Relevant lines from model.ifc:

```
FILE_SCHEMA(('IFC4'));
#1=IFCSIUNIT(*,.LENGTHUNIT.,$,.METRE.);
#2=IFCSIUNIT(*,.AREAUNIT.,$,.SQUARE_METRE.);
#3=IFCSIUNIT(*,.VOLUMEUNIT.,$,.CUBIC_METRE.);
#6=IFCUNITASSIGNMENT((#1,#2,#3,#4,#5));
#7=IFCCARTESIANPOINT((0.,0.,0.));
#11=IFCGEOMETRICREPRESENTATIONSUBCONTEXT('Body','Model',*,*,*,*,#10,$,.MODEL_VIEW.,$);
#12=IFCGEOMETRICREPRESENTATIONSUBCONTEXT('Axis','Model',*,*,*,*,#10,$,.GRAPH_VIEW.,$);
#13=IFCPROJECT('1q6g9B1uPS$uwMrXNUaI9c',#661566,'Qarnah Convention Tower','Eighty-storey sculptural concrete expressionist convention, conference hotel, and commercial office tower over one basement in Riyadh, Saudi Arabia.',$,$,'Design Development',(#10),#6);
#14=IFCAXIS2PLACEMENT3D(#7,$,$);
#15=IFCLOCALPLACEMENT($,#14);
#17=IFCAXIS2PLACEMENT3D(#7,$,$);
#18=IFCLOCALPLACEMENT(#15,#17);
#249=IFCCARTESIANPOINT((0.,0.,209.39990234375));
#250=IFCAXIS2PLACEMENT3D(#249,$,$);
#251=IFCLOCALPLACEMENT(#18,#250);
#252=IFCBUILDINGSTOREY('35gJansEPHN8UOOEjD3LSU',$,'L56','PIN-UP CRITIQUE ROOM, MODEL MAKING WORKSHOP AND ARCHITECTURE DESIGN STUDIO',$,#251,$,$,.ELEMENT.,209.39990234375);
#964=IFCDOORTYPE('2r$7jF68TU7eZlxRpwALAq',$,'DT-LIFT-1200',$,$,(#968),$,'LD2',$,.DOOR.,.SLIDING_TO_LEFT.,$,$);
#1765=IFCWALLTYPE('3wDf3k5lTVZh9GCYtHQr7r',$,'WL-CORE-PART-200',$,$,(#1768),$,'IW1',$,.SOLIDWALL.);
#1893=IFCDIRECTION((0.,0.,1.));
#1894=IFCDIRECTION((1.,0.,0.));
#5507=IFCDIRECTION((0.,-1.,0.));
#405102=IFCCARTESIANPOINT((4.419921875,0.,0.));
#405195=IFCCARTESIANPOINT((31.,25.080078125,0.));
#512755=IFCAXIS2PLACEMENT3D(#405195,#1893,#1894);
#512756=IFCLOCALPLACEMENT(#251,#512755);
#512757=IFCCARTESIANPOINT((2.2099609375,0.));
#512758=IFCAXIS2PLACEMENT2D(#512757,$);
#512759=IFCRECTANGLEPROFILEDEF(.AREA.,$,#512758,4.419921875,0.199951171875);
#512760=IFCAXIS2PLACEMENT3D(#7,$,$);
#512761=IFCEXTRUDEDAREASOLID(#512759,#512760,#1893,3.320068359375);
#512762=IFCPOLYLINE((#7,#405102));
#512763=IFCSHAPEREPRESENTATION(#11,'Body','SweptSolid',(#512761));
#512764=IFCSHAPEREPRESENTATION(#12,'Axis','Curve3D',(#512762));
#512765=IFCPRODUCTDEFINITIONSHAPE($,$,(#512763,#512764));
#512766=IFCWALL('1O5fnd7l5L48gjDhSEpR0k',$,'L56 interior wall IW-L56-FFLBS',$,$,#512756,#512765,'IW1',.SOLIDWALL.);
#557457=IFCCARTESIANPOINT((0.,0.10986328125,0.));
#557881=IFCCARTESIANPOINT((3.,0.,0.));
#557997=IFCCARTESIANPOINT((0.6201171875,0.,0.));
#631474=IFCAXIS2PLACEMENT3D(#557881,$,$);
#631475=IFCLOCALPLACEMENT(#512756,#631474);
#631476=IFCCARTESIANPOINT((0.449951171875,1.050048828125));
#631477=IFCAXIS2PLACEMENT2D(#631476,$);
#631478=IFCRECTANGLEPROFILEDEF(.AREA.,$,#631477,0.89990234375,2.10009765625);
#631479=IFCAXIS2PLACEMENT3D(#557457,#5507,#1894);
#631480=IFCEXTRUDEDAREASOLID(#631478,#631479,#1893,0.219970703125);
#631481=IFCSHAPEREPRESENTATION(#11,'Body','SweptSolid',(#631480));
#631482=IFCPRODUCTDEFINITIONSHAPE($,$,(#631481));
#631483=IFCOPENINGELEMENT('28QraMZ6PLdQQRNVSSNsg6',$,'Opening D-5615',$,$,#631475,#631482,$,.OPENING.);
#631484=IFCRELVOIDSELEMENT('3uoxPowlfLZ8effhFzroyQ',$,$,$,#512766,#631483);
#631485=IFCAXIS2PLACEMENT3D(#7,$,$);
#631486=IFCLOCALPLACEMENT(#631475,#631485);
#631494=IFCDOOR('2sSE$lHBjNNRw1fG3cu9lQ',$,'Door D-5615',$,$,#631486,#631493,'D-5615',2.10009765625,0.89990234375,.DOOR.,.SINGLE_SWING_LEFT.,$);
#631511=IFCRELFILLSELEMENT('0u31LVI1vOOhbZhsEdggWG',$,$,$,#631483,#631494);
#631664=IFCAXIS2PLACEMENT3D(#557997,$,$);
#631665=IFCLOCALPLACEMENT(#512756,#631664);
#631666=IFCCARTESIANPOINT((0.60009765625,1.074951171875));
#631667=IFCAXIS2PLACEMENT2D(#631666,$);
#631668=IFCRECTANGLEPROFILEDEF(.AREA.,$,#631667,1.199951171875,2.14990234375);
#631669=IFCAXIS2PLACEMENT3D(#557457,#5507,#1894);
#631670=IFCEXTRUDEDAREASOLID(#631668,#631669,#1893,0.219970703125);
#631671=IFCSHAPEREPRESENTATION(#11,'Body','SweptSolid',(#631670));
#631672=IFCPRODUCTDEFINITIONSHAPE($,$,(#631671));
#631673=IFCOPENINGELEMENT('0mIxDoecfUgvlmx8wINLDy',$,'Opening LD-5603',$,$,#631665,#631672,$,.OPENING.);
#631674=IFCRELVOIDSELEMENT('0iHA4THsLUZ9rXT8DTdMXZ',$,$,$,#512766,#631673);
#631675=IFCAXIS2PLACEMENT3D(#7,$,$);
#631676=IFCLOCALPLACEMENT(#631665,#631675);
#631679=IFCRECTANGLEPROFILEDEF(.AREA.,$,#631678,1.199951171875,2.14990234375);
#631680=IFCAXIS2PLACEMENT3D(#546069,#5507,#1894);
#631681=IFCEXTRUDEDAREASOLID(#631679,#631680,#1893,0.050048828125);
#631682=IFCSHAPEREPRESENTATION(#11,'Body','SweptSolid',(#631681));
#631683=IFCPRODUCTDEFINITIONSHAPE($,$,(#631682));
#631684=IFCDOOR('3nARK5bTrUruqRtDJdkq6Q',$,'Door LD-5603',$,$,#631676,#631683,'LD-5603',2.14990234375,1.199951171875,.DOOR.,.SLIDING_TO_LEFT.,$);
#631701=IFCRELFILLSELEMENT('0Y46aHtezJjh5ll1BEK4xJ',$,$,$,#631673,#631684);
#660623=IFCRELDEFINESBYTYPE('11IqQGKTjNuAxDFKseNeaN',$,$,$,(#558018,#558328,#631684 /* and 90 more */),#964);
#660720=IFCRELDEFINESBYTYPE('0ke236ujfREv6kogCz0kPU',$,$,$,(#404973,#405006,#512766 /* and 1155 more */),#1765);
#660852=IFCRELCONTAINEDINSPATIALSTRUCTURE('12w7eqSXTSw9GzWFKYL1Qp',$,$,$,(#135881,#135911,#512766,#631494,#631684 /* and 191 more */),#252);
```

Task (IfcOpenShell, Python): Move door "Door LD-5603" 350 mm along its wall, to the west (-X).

```python
import ifcopenshell
import ifcopenshell.api.geometry
import ifcopenshell.util.placement
import ifcopenshell.util.unit

model = ifcopenshell.open("model.ifc")
unit_scale = ifcopenshell.util.unit.calculate_unit_scale(model)

door = model.by_guid("3nARK5bTrUruqRtDJdkq6Q")
opening = door.FillsVoids[0].RelatingOpeningElement
wall = opening.VoidsElements[0].RelatingBuildingElement

wall_matrix = ifcopenshell.util.placement.get_local_placement(wall.ObjectPlacement)
shift = wall_matrix[:3, 0] * -0.35 / unit_scale
before = ifcopenshell.util.placement.get_local_placement(door.ObjectPlacement)[:3, 3].copy()

# The door is placed relative to its opening, so it follows when the opening moves.
matrix = ifcopenshell.util.placement.get_local_placement(opening.ObjectPlacement)
matrix[:3, 3] += shift
ifcopenshell.api.geometry.edit_object_placement(
    model, product=opening, matrix=matrix, is_si=False, should_transform_children=True
)

after = ifcopenshell.util.placement.get_local_placement(door.ObjectPlacement)[:3, 3]
print("door moved by", (after - before).round(3) + 0.0)

model.write("model_updated.ifc")
```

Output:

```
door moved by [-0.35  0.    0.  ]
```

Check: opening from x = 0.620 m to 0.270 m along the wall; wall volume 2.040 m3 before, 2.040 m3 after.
